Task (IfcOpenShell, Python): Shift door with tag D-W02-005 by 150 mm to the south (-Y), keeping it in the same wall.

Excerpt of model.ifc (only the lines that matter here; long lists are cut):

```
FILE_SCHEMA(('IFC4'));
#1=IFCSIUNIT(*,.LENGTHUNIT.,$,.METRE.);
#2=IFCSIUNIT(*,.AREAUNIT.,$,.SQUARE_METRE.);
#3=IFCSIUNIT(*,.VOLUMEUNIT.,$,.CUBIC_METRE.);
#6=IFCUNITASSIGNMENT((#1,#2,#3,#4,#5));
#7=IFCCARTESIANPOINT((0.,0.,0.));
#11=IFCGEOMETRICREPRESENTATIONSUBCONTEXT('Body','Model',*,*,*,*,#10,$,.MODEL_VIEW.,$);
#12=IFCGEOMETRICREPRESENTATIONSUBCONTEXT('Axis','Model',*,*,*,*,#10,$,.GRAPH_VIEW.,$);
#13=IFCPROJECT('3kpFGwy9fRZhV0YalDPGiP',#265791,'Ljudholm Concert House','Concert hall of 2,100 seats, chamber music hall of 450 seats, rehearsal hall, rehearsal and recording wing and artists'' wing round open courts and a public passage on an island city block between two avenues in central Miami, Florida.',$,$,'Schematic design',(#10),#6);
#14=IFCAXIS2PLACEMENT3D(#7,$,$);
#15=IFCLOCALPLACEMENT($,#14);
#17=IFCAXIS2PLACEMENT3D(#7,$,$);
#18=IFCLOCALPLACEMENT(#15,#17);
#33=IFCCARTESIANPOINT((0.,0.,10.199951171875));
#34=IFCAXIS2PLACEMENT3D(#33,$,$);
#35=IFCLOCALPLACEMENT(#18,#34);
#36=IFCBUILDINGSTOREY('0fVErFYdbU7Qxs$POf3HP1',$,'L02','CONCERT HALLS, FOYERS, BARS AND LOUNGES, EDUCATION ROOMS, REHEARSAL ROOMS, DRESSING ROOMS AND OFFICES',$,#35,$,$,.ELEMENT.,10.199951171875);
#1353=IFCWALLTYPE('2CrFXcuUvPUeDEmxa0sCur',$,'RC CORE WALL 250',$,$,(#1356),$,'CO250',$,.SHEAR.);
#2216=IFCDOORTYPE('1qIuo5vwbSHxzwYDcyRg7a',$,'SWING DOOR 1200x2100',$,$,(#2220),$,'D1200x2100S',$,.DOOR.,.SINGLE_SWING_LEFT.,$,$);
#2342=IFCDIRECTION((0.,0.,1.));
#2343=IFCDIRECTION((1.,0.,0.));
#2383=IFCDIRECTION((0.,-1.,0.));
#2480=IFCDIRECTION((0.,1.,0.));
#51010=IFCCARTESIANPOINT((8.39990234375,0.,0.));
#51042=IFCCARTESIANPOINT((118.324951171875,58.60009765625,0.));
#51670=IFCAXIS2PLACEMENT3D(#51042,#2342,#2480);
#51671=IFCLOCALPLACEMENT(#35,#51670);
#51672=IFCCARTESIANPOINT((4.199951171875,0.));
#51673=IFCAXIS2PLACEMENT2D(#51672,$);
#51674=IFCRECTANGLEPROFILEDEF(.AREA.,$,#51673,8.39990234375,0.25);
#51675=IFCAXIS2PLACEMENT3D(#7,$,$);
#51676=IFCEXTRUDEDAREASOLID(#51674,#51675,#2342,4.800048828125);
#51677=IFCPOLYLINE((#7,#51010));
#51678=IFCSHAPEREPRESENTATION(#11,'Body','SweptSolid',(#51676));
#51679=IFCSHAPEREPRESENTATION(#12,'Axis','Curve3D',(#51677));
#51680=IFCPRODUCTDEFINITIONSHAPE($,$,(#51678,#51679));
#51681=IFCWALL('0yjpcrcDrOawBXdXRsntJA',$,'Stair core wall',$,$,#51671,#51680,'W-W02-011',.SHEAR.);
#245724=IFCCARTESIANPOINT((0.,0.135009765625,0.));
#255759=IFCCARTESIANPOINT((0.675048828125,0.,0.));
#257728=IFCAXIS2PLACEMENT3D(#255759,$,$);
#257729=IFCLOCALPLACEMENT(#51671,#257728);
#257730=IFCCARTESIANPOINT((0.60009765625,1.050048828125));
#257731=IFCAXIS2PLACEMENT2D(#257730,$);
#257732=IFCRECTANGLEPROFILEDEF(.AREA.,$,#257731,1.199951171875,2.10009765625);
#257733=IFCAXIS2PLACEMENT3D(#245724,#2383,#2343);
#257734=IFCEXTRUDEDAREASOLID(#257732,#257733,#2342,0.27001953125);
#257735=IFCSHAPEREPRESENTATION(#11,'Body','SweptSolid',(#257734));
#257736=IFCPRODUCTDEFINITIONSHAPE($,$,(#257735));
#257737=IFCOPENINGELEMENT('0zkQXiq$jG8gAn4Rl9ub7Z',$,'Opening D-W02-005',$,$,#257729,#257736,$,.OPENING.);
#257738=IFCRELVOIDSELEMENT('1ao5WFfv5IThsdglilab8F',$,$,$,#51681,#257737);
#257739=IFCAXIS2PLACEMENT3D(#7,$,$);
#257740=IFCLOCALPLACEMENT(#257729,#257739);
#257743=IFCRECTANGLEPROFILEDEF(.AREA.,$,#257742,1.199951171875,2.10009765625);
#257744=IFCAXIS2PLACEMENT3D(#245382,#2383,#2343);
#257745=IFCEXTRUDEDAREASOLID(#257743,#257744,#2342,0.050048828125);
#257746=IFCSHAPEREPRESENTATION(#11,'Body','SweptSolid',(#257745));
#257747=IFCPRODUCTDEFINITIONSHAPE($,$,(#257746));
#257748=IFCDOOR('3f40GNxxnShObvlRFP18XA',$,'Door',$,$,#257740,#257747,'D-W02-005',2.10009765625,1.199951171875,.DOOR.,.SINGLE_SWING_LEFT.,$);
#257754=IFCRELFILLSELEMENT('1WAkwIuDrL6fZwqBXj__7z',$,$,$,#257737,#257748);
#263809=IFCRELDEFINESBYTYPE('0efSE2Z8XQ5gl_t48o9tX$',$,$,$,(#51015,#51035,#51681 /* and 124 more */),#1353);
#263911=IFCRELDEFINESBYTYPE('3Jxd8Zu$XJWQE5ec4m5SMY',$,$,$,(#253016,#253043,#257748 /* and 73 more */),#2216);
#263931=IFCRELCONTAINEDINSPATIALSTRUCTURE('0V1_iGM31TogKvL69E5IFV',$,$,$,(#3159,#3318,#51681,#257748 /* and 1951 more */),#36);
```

```python
import ifcopenshell
import ifcopenshell.api.geometry
import ifcopenshell.util.placement

model = ifcopenshell.open("model.ifc")

door = model.by_guid("3f40GNxxnShObvlRFP18XA")
opening = door.FillsVoids[0].RelatingOpeningElement
wall = opening.VoidsElements[0].RelatingBuildingElement

wall_matrix = ifcopenshell.util.placement.get_local_placement(wall.ObjectPlacement)
shift = wall_matrix[:3, 0] * -0.15
before = ifcopenshell.util.placement.get_local_placement(door.ObjectPlacement)[:3, 3].copy()

# The door is placed relative to its opening, so it follows when the opening moves.
matrix = ifcopenshell.util.placement.get_local_placement(opening.ObjectPlacement)
matrix[:3, 3] += shift
ifcopenshell.api.geometry.edit_object_placement(
    model, product=opening, matrix=matrix, is_si=False, should_transform_children=True
)

after = ifcopenshell.util.placement.get_local_placement(door.ObjectPlacement)[:3, 3]
print("door moved by", (after - before).round(3) + 0.0)

model.write("model_v2.ifc")
```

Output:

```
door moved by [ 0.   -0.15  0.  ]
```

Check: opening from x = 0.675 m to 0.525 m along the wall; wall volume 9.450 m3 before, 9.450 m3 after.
